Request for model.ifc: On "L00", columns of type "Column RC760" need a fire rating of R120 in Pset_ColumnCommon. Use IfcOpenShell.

First a look at what the model holds.

```python
import ifcopenshell
import ifcopenshell.util.element

model = ifcopenshell.open("model.ifc")
print(model.schema)
storey = next(s for s in model.by_type("IfcBuildingStorey") if s.Name == "L00")
columns = [e for e in ifcopenshell.util.element.get_decomposition(storey) if e.is_a("IfcColumn")]
seen = {}
for e in columns:
    element_type = ifcopenshell.util.element.get_type(e)
    key = (element_type.Name if element_type != e and element_type else None, ifcopenshell.util.element.get_pset(e, "Pset_ColumnCommon", "FireRating"))
    seen[key] = seen.get(key, 0) + 1
for (name, value), count in sorted(seen.items(), key=str):
    print(count, "x", name, "|", value)
```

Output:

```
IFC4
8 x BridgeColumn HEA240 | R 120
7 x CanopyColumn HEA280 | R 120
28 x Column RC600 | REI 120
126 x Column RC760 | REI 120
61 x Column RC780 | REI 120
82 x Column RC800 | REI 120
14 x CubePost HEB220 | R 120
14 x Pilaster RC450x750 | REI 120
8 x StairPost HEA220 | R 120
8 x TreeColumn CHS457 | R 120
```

```python
import ifcopenshell
import ifcopenshell.api.pset
import ifcopenshell.util.element

model = ifcopenshell.open("model.ifc")

storey = next(s for s in model.by_type("IfcBuildingStorey") if s.Name == "L00")
columns = [e for e in ifcopenshell.util.element.get_decomposition(storey) if e.is_a("IfcColumn")]

count = 0
for e in columns:
    element_type = ifcopenshell.util.element.get_type(e)
    if element_type in (None, e) or element_type.Name != "Column RC760":
        continue
    # add_pset returns the element's existing set when there is one.
    pset = ifcopenshell.api.pset.add_pset(model, product=e, name="Pset_ColumnCommon")
    ifcopenshell.api.pset.edit_pset(model, pset=pset, properties={"FireRating": "R120"})
    count += 1

print(count, "columns updated")

model.write("model_rev.ifc")
```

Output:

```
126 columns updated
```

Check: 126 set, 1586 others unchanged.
